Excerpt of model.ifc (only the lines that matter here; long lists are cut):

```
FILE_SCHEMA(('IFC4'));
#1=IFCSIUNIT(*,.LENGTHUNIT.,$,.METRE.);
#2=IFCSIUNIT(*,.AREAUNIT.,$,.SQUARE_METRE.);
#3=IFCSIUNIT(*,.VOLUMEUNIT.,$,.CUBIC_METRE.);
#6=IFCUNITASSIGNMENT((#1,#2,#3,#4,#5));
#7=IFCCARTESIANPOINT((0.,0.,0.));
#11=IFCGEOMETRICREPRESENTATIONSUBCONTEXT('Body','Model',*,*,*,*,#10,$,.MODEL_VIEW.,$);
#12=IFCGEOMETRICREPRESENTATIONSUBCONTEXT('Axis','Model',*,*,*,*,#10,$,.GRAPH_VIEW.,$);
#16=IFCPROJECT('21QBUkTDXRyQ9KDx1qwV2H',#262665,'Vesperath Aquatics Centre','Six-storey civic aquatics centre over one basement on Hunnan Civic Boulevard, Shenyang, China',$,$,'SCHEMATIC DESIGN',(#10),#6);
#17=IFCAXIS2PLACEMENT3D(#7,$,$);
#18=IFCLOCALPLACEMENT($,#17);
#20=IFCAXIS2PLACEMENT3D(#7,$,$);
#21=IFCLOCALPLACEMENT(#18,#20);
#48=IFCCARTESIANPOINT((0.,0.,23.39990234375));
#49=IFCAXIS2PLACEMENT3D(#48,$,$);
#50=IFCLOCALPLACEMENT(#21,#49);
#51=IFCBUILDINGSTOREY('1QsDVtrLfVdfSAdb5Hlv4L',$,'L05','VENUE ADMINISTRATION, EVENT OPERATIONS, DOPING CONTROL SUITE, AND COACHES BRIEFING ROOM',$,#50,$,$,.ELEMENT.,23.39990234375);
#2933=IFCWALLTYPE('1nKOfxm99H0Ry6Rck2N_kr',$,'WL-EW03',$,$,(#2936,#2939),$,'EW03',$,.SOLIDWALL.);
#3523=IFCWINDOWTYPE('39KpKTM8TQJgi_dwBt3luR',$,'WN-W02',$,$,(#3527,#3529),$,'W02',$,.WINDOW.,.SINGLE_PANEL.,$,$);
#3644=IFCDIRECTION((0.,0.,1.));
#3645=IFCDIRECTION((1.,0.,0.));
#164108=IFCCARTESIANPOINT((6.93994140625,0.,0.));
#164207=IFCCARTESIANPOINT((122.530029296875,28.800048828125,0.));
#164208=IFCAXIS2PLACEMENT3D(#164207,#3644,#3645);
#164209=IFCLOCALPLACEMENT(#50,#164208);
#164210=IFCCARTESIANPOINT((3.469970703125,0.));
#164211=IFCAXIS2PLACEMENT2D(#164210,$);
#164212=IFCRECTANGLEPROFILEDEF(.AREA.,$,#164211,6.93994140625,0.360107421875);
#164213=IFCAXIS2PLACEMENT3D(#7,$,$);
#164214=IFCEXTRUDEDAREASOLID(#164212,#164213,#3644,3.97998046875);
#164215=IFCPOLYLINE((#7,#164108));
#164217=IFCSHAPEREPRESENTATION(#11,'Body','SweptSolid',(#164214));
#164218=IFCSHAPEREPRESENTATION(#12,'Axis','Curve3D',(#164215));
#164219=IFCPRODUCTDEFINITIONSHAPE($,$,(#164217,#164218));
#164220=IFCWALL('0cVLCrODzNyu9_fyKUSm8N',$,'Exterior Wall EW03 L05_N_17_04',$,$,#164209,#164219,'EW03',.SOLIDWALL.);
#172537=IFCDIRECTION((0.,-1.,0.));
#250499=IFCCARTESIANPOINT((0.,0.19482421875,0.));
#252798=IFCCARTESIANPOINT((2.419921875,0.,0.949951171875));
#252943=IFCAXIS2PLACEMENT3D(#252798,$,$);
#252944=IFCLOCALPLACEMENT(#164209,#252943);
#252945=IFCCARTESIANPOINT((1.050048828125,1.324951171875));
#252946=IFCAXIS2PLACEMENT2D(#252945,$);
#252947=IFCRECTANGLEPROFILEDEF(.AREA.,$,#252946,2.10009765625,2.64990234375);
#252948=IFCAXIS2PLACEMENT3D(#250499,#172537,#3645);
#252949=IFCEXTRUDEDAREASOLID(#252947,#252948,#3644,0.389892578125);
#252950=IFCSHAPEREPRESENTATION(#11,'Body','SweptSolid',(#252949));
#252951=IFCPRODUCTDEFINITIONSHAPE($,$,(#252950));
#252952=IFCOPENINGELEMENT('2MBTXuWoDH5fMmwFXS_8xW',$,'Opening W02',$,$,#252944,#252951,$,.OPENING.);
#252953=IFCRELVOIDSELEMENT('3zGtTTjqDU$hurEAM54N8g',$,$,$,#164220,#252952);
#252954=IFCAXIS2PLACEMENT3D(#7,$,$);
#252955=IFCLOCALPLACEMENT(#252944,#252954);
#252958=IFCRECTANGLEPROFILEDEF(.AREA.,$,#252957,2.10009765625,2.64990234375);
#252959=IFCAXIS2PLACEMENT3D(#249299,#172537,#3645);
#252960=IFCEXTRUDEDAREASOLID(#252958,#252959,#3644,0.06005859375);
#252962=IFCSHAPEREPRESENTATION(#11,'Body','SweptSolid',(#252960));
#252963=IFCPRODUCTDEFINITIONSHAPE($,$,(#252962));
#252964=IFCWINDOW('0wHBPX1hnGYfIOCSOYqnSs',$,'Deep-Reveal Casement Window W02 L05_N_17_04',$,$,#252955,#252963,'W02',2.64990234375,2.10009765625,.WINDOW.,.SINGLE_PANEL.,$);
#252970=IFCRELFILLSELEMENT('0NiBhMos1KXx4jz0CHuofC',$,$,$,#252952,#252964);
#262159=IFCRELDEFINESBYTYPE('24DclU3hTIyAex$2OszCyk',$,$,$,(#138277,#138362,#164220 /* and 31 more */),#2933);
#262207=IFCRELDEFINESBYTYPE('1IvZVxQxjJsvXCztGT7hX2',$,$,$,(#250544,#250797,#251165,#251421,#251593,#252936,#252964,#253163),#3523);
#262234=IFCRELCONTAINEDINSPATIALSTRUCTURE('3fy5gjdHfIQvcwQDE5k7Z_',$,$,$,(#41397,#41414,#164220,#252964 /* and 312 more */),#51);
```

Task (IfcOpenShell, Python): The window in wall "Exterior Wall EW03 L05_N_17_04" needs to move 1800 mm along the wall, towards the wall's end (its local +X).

```python
import ifcopenshell
import ifcopenshell.api.geometry
import ifcopenshell.util.placement

model = ifcopenshell.open("model.ifc")

window = model.by_guid("0wHBPX1hnGYfIOCSOYqnSs")
opening = window.FillsVoids[0].RelatingOpeningElement
wall = opening.VoidsElements[0].RelatingBuildingElement

wall_matrix = ifcopenshell.util.placement.get_local_placement(wall.ObjectPlacement)
shift = wall_matrix[:3, 0] * 1.8
before = ifcopenshell.util.placement.get_local_placement(window.ObjectPlacement)[:3, 3].copy()

# The window is placed relative to its opening, so it follows when the opening moves.
matrix = ifcopenshell.util.placement.get_local_placement(opening.ObjectPlacement)
matrix[:3, 3] += shift
ifcopenshell.api.geometry.edit_object_placement(
    model, product=opening, matrix=matrix, is_si=False, should_transform_children=True
)

after = ifcopenshell.util.placement.get_local_placement(window.ObjectPlacement)[:3, 3]
print("window moved by", (after - before).round(3) + 0.0)

model.write("model_rev.ifc")
```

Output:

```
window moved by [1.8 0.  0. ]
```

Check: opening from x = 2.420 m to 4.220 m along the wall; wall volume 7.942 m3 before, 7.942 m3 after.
